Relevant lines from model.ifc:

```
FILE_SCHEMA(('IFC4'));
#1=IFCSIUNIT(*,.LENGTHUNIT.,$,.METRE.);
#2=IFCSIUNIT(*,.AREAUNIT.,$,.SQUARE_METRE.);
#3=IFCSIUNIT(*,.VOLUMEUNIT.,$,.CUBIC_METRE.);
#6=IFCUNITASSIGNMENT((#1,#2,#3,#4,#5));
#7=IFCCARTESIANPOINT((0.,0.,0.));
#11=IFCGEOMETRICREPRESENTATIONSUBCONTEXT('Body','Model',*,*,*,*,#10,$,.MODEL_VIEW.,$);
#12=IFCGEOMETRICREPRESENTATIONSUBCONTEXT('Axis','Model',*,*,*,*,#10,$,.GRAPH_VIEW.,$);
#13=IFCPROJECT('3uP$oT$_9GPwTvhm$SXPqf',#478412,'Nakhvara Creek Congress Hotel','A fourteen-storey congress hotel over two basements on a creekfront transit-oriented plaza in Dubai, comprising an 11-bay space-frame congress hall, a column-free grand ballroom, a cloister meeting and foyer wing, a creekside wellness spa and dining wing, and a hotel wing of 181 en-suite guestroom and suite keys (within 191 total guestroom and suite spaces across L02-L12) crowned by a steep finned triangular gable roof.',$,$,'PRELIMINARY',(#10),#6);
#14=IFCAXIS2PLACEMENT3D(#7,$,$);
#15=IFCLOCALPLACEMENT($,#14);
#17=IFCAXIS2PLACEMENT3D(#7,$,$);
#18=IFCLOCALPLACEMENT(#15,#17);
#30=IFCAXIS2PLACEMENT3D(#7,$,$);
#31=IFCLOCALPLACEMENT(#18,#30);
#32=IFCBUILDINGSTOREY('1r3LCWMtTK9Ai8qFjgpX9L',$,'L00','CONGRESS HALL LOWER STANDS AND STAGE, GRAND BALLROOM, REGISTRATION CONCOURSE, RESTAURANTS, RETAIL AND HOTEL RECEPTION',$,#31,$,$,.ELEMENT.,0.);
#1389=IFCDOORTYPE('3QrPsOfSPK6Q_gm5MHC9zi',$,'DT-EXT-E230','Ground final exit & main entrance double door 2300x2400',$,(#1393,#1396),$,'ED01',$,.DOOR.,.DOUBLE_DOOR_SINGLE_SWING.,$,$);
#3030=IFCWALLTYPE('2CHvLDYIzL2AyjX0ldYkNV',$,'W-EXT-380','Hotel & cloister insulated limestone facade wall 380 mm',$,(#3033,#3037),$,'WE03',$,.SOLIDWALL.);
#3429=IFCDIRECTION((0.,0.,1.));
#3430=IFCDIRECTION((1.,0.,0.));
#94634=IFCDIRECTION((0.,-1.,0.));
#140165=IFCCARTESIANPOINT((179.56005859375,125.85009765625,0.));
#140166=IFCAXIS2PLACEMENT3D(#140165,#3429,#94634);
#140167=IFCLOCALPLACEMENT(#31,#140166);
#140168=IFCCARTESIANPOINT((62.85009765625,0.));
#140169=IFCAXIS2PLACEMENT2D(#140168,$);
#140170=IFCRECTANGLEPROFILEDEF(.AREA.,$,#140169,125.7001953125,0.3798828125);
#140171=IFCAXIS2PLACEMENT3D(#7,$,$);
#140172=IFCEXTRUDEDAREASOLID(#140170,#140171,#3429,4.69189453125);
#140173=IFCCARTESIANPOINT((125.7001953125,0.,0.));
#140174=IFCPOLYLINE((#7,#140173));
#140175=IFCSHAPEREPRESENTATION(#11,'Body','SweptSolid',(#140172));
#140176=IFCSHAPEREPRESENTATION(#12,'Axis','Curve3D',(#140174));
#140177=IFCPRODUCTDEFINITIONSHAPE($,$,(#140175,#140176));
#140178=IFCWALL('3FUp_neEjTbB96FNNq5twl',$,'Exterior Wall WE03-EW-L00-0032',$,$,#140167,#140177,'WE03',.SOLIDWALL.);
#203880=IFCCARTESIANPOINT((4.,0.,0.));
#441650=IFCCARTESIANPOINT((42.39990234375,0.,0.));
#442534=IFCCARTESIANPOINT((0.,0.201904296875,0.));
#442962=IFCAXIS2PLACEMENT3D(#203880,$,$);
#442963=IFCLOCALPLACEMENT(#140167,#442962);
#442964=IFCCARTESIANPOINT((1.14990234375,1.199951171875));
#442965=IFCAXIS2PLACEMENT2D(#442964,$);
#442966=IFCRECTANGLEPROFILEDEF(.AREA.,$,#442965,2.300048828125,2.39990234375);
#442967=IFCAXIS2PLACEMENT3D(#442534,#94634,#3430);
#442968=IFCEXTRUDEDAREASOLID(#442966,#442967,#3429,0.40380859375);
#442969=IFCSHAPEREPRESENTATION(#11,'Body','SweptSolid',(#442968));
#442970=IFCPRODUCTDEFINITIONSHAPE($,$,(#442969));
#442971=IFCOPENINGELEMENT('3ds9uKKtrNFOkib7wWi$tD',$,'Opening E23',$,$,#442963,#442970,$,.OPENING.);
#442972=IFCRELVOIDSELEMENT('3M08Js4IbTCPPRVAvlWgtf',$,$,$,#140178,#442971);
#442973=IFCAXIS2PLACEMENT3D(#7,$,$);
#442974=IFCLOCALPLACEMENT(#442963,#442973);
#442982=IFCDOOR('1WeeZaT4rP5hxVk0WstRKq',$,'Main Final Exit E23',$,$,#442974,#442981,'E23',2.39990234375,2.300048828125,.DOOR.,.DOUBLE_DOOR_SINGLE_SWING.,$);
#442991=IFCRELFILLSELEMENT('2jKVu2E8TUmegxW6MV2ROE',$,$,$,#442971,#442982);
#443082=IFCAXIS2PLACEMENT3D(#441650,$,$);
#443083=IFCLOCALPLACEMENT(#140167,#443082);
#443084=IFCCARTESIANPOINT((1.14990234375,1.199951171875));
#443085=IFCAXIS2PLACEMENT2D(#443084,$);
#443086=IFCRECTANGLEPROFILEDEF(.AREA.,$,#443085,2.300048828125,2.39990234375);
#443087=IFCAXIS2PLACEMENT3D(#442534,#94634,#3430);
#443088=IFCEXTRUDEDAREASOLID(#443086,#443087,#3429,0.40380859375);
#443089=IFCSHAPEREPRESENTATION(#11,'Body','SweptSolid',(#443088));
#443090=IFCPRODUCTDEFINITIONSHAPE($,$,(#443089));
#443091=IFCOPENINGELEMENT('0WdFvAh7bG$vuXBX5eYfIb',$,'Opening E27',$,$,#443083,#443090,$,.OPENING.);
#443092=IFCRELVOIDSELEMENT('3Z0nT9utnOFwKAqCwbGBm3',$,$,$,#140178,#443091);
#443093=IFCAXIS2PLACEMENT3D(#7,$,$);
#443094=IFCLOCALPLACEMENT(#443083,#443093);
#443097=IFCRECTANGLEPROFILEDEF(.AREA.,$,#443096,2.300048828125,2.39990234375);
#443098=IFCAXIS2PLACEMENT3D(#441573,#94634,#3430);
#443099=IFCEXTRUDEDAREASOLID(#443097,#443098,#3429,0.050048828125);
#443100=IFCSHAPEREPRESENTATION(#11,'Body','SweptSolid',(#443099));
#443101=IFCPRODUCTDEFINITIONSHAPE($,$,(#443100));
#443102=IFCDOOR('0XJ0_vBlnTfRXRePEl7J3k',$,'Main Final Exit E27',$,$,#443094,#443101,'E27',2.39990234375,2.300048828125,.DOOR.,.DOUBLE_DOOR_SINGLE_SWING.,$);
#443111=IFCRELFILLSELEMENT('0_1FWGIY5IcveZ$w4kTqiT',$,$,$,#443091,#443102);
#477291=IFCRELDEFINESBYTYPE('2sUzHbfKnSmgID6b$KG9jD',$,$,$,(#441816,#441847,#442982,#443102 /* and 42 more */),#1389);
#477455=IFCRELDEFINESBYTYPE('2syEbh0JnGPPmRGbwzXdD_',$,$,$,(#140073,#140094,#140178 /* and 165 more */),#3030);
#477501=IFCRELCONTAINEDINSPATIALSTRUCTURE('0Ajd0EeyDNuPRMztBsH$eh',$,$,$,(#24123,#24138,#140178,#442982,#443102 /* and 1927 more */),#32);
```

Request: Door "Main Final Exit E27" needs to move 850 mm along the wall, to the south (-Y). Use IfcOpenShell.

```python
import ifcopenshell
import ifcopenshell.api.geometry
import ifcopenshell.util.placement

model = ifcopenshell.open("model.ifc")

door = model.by_guid("0XJ0_vBlnTfRXRePEl7J3k")
opening = door.FillsVoids[0].RelatingOpeningElement
wall = opening.VoidsElements[0].RelatingBuildingElement

wall_matrix = ifcopenshell.util.placement.get_local_placement(wall.ObjectPlacement)
shift = wall_matrix[:3, 0] * 0.85
before = ifcopenshell.util.placement.get_local_placement(door.ObjectPlacement)[:3, 3].copy()

# The door is placed relative to its opening, so it follows when the opening moves.
matrix = ifcopenshell.util.placement.get_local_placement(opening.ObjectPlacement)
matrix[:3, 3] += shift
ifcopenshell.api.geometry.edit_object_placement(
    model, product=opening, matrix=matrix, is_si=False, should_transform_children=True
)

after = ifcopenshell.util.placement.get_local_placement(door.ObjectPlacement)[:3, 3]
print("door moved by", (after - before).round(3) + 0.0)

model.write("model_edited.ifc")
```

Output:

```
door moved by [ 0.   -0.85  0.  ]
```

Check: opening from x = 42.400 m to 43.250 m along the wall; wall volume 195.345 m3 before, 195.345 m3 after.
